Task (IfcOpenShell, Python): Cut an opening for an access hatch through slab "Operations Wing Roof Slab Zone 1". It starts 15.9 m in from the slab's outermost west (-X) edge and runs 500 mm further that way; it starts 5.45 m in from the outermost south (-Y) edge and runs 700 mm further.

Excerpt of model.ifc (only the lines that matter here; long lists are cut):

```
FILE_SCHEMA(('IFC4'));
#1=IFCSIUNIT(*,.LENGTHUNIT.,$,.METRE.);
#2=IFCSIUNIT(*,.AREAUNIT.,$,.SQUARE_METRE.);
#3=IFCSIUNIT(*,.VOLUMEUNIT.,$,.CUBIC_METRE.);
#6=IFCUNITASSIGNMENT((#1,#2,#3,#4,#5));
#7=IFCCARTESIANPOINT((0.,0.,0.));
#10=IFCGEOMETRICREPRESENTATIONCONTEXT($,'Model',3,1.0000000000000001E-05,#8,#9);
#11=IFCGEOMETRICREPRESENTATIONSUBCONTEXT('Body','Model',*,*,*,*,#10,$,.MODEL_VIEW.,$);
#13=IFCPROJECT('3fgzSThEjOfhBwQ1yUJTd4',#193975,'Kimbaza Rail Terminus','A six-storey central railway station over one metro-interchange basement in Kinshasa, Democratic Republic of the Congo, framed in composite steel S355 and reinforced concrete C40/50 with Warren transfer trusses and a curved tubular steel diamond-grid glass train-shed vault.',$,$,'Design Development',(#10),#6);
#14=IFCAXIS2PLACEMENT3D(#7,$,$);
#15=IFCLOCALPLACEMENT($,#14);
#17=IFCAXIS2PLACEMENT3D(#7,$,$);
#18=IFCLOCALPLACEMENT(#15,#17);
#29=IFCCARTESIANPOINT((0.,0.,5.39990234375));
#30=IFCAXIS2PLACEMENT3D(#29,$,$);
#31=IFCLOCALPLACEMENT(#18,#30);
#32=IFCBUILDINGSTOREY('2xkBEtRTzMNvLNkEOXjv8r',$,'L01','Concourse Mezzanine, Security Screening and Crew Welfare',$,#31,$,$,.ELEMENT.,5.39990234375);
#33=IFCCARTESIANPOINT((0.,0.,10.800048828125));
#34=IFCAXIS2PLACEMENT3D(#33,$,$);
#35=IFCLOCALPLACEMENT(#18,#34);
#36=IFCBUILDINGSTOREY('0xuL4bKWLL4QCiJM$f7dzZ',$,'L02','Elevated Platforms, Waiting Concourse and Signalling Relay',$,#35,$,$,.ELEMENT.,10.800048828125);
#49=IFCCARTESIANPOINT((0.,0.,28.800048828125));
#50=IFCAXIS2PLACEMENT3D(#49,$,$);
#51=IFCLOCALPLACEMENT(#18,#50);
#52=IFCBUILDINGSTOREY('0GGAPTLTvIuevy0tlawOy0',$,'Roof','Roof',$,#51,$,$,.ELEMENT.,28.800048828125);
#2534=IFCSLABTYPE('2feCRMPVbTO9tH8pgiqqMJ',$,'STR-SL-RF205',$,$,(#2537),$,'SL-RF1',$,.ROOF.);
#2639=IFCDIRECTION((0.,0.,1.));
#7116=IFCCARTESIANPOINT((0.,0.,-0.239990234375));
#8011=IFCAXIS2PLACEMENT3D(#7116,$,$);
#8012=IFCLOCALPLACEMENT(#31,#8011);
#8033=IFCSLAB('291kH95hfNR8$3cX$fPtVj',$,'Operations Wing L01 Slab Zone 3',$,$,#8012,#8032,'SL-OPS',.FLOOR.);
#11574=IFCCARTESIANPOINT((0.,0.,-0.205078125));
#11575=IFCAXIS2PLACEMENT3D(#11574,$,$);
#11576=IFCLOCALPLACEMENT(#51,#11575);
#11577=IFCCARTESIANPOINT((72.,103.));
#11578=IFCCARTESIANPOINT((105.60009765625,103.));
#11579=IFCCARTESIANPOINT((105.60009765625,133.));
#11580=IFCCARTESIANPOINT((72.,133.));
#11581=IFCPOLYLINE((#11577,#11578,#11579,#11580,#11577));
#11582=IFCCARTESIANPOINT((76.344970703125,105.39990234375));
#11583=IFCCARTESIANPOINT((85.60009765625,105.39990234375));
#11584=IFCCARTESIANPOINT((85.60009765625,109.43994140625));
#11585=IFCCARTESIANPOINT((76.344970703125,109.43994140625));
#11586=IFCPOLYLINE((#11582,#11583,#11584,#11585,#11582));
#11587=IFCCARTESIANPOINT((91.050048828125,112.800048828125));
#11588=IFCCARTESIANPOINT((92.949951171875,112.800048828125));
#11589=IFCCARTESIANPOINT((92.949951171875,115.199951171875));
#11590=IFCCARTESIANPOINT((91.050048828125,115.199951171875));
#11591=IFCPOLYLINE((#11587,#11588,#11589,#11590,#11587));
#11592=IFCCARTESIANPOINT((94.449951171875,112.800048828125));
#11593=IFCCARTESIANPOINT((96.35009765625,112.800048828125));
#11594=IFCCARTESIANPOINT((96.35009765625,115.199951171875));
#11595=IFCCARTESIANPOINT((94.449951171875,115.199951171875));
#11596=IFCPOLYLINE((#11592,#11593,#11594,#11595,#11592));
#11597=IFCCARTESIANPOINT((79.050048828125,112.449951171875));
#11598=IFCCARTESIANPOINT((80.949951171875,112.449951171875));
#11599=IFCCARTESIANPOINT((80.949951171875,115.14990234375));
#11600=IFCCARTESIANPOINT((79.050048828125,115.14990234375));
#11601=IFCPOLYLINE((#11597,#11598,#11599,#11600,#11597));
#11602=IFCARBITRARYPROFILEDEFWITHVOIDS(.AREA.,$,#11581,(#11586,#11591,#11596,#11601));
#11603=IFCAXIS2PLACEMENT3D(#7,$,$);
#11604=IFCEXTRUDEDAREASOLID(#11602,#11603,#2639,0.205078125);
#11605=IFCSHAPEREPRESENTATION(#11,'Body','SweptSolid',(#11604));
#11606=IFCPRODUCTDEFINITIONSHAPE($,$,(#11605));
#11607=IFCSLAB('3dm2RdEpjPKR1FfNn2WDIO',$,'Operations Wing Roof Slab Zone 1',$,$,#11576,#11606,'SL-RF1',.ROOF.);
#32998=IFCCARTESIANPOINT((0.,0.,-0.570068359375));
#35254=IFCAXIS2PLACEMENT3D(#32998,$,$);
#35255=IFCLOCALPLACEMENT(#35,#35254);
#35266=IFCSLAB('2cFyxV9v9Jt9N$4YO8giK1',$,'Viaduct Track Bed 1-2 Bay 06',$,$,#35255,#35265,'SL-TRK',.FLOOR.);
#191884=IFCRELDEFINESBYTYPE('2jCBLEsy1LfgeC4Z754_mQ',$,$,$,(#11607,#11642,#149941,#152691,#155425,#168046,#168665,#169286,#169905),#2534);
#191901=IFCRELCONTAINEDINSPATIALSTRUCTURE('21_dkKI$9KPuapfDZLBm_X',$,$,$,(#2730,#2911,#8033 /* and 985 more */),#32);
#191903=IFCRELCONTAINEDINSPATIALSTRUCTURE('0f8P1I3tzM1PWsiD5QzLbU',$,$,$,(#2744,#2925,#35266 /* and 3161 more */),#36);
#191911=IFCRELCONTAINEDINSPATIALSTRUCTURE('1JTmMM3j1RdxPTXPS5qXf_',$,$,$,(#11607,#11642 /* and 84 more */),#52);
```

```python
import numpy as np
import ifcopenshell
import ifcopenshell.api.feature
import ifcopenshell.api.geometry
import ifcopenshell.api.root
import ifcopenshell.geom
import ifcopenshell.util.placement
import ifcopenshell.util.representation
import ifcopenshell.util.shape
import ifcopenshell.util.unit

model = ifcopenshell.open("model.ifc")
unit_scale = ifcopenshell.util.unit.calculate_unit_scale(model)
settings = ifcopenshell.geom.settings()


def volume(element):
    """Net volume in cubic metres, openings subtracted."""
    shape = ifcopenshell.geom.create_shape(settings, element)
    return ifcopenshell.util.shape.get_volume(shape.geometry)


slab = model.by_guid("3dm2RdEpjPKR1FfNn2WDIO")
before = volume(slab)

# Extent in the slab's own axes, in metres. The edges named are its -X and -Y sides.
slab_shape = ifcopenshell.geom.create_shape(settings, slab)
vertices = ifcopenshell.util.shape.get_vertices(slab_shape.geometry)
x_min, y_min, bottom = vertices.min(axis=0)
top = vertices[:, 2].max()

opening = ifcopenshell.api.root.create_entity(model, ifc_class="IfcOpeningElement", name="Access hatch opening", predefined_type="OPENING")
context = ifcopenshell.util.representation.get_context(model, "Model", "Body", "MODEL_VIEW")
width, depth = 0.5, 0.7
outline = [(0.0, 0.0), (width, 0.0), (width, depth), (0.0, depth), (0.0, 0.0)]
# Overshoot both faces by 50 mm so the cut is clean.
shape = ifcopenshell.api.geometry.add_slab_representation(
    model, context=context, depth=top - bottom + 0.1, polyline=outline
)
ifcopenshell.api.geometry.assign_representation(model, product=opening, representation=shape)

matrix = ifcopenshell.util.placement.get_local_placement(slab.ObjectPlacement)
matrix[:, 3] = matrix @ np.append(np.array([x_min + 15.9, y_min + 5.45, bottom - 0.05]) / unit_scale, 1.0)
ifcopenshell.api.geometry.edit_object_placement(model, product=opening, matrix=matrix, is_si=False)
ifcopenshell.api.feature.add_feature(model, feature=opening, element=slab)

after = volume(slab)

print(f"slab volume {before:.3f} -> {after:.3f} m3")

model.write("model_updated.ifc")
```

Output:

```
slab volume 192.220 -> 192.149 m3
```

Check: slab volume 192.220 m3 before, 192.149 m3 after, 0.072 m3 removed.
